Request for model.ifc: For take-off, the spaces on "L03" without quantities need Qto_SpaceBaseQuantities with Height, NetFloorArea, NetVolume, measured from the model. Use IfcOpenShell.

First a look at what the model holds.

```python
import ifcopenshell
import ifcopenshell.util.element
import ifcopenshell.util.unit

model = ifcopenshell.open("model.ifc")
print(model.schema)
for unit_type in ("LENGTHUNIT", "AREAUNIT", "VOLUMEUNIT"):
    print(unit_type, ifcopenshell.util.unit.calculate_unit_scale(model, unit_type))
storey = next(s for s in model.by_type("IfcBuildingStorey") if s.Name == "L03")
spaces = [e for e in ifcopenshell.util.element.get_decomposition(storey) if e.is_a("IfcSpace")]
for e in sorted(spaces, key=lambda e: e.id()):
    print(e.id(), e.is_a(), e.Name, list(ifcopenshell.util.element.get_psets(e, qtos_only=True)), sep=" | ")
```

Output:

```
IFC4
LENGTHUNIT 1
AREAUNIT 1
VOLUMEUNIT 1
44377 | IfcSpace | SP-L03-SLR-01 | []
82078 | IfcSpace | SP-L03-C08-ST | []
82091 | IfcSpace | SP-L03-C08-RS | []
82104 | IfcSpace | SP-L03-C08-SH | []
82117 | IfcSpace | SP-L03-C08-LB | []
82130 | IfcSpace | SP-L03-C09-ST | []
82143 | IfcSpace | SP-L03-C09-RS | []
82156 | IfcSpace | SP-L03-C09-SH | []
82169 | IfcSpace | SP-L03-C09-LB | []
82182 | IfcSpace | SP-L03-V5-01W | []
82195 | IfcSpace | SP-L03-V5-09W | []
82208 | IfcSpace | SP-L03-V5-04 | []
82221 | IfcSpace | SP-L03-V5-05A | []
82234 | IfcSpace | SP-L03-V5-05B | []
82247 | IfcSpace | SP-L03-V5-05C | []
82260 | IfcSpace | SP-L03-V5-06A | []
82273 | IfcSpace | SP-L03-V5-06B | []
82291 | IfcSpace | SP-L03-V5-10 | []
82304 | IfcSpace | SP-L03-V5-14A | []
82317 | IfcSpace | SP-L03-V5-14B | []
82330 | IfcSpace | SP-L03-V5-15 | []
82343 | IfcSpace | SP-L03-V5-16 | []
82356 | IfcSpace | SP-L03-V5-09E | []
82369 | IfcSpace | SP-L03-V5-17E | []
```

```python
import ifcopenshell
import ifcopenshell.api.pset
import ifcopenshell.geom
import ifcopenshell.util.element
import ifcopenshell.util.shape
import ifcopenshell.util.unit

model = ifcopenshell.open("model.ifc")
unit_scale = ifcopenshell.util.unit.calculate_unit_scale(model)
area_scale = ifcopenshell.util.unit.calculate_unit_scale(model, "AREAUNIT")
volume_scale = ifcopenshell.util.unit.calculate_unit_scale(model, "VOLUMEUNIT")
settings = ifcopenshell.geom.settings()

storey = next(s for s in model.by_type("IfcBuildingStorey") if s.Name == "L03")
spaces = [e for e in ifcopenshell.util.element.get_decomposition(storey) if e.is_a("IfcSpace")]

for e in sorted(spaces, key=lambda e: e.id()):
    if ifcopenshell.util.element.get_psets(e, qtos_only=True, should_inherit=False):
        continue
    # Geometry comes back in metres, in the element's own axes.
    shape = ifcopenshell.geom.create_shape(settings, e)
    values = {
        "Height": ifcopenshell.util.shape.get_z(shape.geometry) / unit_scale,
        "NetFloorArea": ifcopenshell.util.shape.get_footprint_area(shape.geometry) / area_scale,
        "NetVolume": ifcopenshell.util.shape.get_volume(shape.geometry) / volume_scale,
    }
    qto = ifcopenshell.api.pset.add_qto(model, product=e, name="Qto_SpaceBaseQuantities")
    ifcopenshell.api.pset.edit_qto(model, qto=qto, properties=values)
    print(e.id(), {k: round(v, 3) for k, v in values.items()})

model.write("model-out.ifc")
```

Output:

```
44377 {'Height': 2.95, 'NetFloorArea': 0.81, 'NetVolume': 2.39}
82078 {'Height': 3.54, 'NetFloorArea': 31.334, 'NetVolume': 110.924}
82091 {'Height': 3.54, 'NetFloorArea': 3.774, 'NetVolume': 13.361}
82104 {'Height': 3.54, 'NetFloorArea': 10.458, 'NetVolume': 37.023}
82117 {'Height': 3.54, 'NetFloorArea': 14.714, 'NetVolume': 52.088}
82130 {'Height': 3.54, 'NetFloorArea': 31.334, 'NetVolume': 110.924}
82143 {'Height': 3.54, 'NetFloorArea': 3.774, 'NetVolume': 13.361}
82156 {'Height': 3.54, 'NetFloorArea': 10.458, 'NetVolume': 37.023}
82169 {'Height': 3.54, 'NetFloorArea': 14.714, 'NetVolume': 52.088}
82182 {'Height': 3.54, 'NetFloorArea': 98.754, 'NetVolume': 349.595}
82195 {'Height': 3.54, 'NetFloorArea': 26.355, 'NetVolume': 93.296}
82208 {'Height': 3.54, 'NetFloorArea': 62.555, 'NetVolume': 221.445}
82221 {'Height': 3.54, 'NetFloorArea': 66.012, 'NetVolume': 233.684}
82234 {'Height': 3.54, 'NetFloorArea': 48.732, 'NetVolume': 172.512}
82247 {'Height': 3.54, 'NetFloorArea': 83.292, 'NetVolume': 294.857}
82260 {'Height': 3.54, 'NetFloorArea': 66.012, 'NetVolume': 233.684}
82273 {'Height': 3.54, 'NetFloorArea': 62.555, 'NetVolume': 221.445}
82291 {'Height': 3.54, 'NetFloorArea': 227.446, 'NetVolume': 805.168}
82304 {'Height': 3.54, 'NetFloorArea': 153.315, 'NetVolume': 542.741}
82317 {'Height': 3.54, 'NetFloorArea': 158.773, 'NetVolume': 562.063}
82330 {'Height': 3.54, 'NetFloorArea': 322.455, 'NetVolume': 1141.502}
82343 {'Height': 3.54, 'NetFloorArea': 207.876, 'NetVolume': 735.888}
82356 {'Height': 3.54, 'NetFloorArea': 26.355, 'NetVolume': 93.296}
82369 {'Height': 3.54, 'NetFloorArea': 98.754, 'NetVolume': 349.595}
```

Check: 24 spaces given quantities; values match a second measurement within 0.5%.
